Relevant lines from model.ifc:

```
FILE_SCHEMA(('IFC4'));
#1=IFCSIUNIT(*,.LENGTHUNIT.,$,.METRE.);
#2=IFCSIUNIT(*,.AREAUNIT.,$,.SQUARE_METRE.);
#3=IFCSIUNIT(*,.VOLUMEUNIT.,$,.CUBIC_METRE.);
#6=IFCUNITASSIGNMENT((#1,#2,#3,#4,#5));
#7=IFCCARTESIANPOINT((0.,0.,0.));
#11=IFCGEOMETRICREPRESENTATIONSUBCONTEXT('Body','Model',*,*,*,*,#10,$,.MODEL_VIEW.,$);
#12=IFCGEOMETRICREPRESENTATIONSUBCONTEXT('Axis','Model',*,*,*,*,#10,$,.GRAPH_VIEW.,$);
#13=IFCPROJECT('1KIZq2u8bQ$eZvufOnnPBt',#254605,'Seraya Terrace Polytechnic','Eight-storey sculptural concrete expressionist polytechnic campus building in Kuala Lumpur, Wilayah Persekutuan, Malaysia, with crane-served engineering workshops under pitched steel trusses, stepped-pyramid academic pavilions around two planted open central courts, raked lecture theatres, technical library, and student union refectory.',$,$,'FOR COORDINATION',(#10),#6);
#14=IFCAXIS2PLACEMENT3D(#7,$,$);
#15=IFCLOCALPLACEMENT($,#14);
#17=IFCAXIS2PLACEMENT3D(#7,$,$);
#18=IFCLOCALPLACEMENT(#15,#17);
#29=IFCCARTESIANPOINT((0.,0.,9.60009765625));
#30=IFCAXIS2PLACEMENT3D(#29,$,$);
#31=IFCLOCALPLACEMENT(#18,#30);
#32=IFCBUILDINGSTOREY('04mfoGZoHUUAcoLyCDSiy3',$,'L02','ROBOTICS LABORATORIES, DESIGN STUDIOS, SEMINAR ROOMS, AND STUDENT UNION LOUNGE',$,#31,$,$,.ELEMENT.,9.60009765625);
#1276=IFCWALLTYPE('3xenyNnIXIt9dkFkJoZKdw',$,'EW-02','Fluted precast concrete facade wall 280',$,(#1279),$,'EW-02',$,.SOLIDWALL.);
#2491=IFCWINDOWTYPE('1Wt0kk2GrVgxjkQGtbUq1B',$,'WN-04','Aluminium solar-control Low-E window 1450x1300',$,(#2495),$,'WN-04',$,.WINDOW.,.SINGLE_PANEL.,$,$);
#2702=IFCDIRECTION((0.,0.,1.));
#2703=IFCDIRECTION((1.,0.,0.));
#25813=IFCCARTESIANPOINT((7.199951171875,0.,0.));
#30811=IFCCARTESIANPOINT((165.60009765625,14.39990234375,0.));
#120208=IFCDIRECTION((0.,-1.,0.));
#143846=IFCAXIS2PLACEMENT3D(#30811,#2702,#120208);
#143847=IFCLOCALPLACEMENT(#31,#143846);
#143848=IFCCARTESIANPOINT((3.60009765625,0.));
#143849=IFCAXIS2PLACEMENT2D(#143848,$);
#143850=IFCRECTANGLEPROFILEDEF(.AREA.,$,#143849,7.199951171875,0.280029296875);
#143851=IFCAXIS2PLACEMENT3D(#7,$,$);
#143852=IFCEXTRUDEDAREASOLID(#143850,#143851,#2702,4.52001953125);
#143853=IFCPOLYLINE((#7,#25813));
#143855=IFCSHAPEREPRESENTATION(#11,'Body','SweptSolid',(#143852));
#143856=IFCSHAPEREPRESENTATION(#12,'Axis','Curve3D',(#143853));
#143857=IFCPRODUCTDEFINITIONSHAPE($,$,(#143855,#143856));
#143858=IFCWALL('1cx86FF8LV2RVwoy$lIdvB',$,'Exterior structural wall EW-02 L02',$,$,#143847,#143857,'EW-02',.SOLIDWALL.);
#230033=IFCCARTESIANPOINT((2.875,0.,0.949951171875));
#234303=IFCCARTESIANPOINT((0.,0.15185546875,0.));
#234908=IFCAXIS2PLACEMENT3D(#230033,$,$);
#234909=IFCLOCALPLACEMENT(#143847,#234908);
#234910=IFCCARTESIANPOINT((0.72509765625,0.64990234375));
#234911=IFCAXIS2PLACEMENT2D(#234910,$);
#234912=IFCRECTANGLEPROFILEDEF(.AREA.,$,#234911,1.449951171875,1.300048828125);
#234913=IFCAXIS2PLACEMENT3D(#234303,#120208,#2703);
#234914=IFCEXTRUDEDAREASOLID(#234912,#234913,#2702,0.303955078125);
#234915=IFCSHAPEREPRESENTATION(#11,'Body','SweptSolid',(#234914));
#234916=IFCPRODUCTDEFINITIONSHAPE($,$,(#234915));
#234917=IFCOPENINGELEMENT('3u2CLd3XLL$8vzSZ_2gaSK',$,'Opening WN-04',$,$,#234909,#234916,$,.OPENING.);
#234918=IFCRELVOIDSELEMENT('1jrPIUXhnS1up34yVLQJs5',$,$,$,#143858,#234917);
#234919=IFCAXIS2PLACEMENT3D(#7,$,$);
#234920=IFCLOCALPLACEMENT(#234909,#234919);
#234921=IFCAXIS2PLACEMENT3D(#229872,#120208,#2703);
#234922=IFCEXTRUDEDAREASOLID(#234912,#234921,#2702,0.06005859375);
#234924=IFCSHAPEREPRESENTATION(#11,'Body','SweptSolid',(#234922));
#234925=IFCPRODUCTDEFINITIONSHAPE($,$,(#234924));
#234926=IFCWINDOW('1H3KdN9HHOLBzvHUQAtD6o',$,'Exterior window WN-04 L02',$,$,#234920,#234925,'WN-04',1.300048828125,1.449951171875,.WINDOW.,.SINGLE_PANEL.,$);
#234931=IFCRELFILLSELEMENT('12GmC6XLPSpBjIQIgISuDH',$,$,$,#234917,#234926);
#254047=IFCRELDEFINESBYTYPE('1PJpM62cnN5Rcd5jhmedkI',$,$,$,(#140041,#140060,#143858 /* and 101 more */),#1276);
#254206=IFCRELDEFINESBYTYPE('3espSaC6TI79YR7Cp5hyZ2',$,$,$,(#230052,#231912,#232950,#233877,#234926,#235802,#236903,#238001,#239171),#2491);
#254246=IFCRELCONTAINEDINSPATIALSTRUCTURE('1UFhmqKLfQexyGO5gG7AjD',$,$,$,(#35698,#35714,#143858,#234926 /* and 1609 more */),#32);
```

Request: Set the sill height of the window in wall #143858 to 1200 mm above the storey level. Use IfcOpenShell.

```python
import numpy as np
import ifcopenshell
import ifcopenshell.api.geometry
import ifcopenshell.geom
import ifcopenshell.util.element
import ifcopenshell.util.placement
import ifcopenshell.util.shape
import ifcopenshell.util.unit

model = ifcopenshell.open("model.ifc")
unit_scale = ifcopenshell.util.unit.calculate_unit_scale(model)

window = model.by_guid("1H3KdN9HHOLBzvHUQAtD6o")
opening = window.FillsVoids[0].RelatingOpeningElement
storey = ifcopenshell.util.element.get_container(window, ifc_class="IfcBuildingStorey")
level = ifcopenshell.util.placement.get_local_placement(storey.ObjectPlacement)[2, 3]

# The opening's origin need not be at the sill, so measure its lowest point.
shape = ifcopenshell.geom.create_shape(ifcopenshell.geom.settings(), opening)
bottom = ifcopenshell.util.shape.get_shape_bottom_elevation(shape, shape.geometry) / unit_scale
dz = level + 1.2 / unit_scale - bottom

shift = np.array([0.0, 0.0, dz])
# The window is placed relative to its opening, so it follows when the opening moves.
matrix = ifcopenshell.util.placement.get_local_placement(opening.ObjectPlacement)
matrix[:3, 3] += shift
ifcopenshell.api.geometry.edit_object_placement(
    model, product=opening, matrix=matrix, is_si=False, should_transform_children=True
)

print(f"moved by {dz * unit_scale:+.3f} m")

model.write("model_updated.ifc")
```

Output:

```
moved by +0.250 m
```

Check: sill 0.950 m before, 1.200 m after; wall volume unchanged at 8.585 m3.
